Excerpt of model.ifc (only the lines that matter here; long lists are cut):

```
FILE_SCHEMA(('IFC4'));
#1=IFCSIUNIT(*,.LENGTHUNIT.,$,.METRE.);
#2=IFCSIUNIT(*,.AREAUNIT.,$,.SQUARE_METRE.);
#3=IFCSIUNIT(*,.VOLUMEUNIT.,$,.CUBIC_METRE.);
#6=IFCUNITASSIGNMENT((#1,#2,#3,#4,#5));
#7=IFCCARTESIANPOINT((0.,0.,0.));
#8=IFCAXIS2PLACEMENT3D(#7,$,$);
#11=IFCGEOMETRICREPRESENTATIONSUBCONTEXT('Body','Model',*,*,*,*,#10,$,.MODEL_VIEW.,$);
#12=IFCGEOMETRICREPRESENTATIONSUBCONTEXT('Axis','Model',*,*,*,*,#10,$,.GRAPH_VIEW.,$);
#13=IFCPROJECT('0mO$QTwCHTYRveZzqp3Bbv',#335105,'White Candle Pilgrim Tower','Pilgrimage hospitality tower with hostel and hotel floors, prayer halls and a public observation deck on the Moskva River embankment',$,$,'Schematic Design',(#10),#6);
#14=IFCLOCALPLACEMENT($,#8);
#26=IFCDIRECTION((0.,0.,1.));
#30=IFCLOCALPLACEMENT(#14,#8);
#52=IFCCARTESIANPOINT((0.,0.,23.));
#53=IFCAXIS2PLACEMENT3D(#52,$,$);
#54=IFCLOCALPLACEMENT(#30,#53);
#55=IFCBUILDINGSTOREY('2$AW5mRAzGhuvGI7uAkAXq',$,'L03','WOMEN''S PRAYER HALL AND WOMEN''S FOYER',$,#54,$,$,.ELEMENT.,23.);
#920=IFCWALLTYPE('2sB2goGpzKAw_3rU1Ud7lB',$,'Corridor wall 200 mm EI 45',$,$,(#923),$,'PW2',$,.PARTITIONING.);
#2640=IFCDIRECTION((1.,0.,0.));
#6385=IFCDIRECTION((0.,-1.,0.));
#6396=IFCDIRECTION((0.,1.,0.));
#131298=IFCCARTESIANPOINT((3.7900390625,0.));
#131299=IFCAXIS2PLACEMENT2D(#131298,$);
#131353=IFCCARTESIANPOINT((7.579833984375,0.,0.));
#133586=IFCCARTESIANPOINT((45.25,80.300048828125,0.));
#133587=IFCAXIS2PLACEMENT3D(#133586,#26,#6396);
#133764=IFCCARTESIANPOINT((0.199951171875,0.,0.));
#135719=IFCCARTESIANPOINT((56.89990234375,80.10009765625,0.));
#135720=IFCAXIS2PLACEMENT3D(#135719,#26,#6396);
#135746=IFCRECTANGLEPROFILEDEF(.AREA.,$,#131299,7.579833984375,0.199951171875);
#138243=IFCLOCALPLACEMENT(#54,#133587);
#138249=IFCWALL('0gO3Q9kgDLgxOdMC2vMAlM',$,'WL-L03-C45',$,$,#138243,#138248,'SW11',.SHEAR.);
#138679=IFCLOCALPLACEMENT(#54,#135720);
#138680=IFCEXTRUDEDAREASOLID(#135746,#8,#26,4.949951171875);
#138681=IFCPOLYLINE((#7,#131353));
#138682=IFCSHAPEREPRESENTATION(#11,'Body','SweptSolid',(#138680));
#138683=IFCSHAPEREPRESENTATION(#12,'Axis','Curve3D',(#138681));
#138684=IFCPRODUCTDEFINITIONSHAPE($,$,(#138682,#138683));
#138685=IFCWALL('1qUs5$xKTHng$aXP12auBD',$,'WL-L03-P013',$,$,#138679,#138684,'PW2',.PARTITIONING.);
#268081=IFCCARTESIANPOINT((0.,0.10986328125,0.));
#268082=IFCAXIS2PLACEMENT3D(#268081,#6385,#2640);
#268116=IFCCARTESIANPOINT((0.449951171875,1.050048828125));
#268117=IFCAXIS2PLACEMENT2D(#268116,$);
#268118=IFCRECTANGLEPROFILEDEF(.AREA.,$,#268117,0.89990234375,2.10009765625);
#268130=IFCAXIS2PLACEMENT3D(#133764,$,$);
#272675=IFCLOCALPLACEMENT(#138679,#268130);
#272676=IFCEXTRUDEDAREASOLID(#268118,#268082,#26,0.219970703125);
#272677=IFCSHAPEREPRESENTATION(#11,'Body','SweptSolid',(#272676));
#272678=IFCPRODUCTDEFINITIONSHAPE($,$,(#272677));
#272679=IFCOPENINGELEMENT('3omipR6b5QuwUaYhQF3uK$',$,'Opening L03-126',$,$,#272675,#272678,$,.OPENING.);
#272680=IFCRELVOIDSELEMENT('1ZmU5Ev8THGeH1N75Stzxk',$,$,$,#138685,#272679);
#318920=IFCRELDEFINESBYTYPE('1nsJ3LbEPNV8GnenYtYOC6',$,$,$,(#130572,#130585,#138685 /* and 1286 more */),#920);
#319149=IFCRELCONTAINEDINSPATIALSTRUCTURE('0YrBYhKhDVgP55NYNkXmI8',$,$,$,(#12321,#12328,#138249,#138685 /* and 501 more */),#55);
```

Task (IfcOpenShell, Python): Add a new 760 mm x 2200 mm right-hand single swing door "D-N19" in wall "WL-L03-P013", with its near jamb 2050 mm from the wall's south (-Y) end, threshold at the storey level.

```python
import numpy as np
import ifcopenshell
import ifcopenshell.api.feature
import ifcopenshell.api.geometry
import ifcopenshell.api.root
import ifcopenshell.api.spatial
import ifcopenshell.geom
import ifcopenshell.util.element
import ifcopenshell.util.placement
import ifcopenshell.util.representation
import ifcopenshell.util.shape
import ifcopenshell.util.unit

model = ifcopenshell.open("model.ifc")
unit_scale = ifcopenshell.util.unit.calculate_unit_scale(model)
settings = ifcopenshell.geom.settings()


def volume(element):
    """Net volume in cubic metres, openings subtracted."""
    shape = ifcopenshell.geom.create_shape(settings, element)
    return ifcopenshell.util.shape.get_volume(shape.geometry)


wall = model.by_id(138685)
storey = ifcopenshell.util.element.get_container(wall, ifc_class="IfcBuildingStorey")
context = ifcopenshell.util.representation.get_context(model, "Model", "Body", "MODEL_VIEW")
before = volume(wall)

width, height, from_end, sill = 0.76, 2.2, 2.05, 0.0  # metres

# The wall runs along its own X axis, and the end named is its -X end.
wall_shape = ifcopenshell.geom.create_shape(settings, wall)
x, y, z = ifcopenshell.util.shape.get_vertices(wall_shape.geometry).T
start = x.min() + from_end
face, thickness = float(y.min()), float(y.max() - y.min())
wall_matrix = ifcopenshell.util.placement.get_local_placement(wall.ObjectPlacement)
level = ifcopenshell.util.placement.get_local_placement(storey.ObjectPlacement)[2, 3]


def in_wall(x, y):
    """Placement at x, y metres in the wall's axes, at sill height."""
    matrix = wall_matrix.copy()
    matrix[:, 3] = wall_matrix @ np.array([x / unit_scale, y / unit_scale, 0.0, 1.0])
    matrix[2, 3] = level + sill / unit_scale
    return matrix


# Opening: a box that overshoots both wall faces by 50 mm.
opening = ifcopenshell.api.root.create_entity(model, ifc_class="IfcOpeningElement", predefined_type="OPENING")
box = ifcopenshell.api.geometry.add_wall_representation(
    model, context=context, length=width, height=height, thickness=thickness + 0.1
)
ifcopenshell.api.geometry.assign_representation(model, product=opening, representation=box)
ifcopenshell.api.geometry.edit_object_placement(model, product=opening, matrix=in_wall(start, face - 0.05), is_si=False)
ifcopenshell.api.feature.add_feature(model, feature=opening, element=wall)

door = ifcopenshell.api.root.create_entity(model, ifc_class="IfcDoor", name="D-N19", predefined_type="DOOR")
door.OverallWidth, door.OverallHeight = width / unit_scale, height / unit_scale
door.OperationType = "SINGLE_SWING_RIGHT"
body = ifcopenshell.api.geometry.add_door_representation(
    model,
    context=context,
    overall_width=door.OverallWidth,
    overall_height=door.OverallHeight,
    operation_type="SINGLE_SWING_RIGHT",
    lining_properties={"LiningDepth": thickness / unit_scale, "ThresholdDepth": thickness / unit_scale},
)
ifcopenshell.api.geometry.assign_representation(model, product=door, representation=body)
ifcopenshell.api.spatial.assign_container(model, products=[door], relating_structure=storey)
ifcopenshell.api.feature.add_filling(model, opening=opening, element=door)

# The lining spans the wall, so the door starts at the wall face.
ifcopenshell.api.geometry.edit_object_placement(model, product=door, matrix=in_wall(start, face), is_si=False)

after = volume(wall)

print(f"wall volume {before:.3f} -> {after:.3f} m3")

model.write("model_v2.ifc")
```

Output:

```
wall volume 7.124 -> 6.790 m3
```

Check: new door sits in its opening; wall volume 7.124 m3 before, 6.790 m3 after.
